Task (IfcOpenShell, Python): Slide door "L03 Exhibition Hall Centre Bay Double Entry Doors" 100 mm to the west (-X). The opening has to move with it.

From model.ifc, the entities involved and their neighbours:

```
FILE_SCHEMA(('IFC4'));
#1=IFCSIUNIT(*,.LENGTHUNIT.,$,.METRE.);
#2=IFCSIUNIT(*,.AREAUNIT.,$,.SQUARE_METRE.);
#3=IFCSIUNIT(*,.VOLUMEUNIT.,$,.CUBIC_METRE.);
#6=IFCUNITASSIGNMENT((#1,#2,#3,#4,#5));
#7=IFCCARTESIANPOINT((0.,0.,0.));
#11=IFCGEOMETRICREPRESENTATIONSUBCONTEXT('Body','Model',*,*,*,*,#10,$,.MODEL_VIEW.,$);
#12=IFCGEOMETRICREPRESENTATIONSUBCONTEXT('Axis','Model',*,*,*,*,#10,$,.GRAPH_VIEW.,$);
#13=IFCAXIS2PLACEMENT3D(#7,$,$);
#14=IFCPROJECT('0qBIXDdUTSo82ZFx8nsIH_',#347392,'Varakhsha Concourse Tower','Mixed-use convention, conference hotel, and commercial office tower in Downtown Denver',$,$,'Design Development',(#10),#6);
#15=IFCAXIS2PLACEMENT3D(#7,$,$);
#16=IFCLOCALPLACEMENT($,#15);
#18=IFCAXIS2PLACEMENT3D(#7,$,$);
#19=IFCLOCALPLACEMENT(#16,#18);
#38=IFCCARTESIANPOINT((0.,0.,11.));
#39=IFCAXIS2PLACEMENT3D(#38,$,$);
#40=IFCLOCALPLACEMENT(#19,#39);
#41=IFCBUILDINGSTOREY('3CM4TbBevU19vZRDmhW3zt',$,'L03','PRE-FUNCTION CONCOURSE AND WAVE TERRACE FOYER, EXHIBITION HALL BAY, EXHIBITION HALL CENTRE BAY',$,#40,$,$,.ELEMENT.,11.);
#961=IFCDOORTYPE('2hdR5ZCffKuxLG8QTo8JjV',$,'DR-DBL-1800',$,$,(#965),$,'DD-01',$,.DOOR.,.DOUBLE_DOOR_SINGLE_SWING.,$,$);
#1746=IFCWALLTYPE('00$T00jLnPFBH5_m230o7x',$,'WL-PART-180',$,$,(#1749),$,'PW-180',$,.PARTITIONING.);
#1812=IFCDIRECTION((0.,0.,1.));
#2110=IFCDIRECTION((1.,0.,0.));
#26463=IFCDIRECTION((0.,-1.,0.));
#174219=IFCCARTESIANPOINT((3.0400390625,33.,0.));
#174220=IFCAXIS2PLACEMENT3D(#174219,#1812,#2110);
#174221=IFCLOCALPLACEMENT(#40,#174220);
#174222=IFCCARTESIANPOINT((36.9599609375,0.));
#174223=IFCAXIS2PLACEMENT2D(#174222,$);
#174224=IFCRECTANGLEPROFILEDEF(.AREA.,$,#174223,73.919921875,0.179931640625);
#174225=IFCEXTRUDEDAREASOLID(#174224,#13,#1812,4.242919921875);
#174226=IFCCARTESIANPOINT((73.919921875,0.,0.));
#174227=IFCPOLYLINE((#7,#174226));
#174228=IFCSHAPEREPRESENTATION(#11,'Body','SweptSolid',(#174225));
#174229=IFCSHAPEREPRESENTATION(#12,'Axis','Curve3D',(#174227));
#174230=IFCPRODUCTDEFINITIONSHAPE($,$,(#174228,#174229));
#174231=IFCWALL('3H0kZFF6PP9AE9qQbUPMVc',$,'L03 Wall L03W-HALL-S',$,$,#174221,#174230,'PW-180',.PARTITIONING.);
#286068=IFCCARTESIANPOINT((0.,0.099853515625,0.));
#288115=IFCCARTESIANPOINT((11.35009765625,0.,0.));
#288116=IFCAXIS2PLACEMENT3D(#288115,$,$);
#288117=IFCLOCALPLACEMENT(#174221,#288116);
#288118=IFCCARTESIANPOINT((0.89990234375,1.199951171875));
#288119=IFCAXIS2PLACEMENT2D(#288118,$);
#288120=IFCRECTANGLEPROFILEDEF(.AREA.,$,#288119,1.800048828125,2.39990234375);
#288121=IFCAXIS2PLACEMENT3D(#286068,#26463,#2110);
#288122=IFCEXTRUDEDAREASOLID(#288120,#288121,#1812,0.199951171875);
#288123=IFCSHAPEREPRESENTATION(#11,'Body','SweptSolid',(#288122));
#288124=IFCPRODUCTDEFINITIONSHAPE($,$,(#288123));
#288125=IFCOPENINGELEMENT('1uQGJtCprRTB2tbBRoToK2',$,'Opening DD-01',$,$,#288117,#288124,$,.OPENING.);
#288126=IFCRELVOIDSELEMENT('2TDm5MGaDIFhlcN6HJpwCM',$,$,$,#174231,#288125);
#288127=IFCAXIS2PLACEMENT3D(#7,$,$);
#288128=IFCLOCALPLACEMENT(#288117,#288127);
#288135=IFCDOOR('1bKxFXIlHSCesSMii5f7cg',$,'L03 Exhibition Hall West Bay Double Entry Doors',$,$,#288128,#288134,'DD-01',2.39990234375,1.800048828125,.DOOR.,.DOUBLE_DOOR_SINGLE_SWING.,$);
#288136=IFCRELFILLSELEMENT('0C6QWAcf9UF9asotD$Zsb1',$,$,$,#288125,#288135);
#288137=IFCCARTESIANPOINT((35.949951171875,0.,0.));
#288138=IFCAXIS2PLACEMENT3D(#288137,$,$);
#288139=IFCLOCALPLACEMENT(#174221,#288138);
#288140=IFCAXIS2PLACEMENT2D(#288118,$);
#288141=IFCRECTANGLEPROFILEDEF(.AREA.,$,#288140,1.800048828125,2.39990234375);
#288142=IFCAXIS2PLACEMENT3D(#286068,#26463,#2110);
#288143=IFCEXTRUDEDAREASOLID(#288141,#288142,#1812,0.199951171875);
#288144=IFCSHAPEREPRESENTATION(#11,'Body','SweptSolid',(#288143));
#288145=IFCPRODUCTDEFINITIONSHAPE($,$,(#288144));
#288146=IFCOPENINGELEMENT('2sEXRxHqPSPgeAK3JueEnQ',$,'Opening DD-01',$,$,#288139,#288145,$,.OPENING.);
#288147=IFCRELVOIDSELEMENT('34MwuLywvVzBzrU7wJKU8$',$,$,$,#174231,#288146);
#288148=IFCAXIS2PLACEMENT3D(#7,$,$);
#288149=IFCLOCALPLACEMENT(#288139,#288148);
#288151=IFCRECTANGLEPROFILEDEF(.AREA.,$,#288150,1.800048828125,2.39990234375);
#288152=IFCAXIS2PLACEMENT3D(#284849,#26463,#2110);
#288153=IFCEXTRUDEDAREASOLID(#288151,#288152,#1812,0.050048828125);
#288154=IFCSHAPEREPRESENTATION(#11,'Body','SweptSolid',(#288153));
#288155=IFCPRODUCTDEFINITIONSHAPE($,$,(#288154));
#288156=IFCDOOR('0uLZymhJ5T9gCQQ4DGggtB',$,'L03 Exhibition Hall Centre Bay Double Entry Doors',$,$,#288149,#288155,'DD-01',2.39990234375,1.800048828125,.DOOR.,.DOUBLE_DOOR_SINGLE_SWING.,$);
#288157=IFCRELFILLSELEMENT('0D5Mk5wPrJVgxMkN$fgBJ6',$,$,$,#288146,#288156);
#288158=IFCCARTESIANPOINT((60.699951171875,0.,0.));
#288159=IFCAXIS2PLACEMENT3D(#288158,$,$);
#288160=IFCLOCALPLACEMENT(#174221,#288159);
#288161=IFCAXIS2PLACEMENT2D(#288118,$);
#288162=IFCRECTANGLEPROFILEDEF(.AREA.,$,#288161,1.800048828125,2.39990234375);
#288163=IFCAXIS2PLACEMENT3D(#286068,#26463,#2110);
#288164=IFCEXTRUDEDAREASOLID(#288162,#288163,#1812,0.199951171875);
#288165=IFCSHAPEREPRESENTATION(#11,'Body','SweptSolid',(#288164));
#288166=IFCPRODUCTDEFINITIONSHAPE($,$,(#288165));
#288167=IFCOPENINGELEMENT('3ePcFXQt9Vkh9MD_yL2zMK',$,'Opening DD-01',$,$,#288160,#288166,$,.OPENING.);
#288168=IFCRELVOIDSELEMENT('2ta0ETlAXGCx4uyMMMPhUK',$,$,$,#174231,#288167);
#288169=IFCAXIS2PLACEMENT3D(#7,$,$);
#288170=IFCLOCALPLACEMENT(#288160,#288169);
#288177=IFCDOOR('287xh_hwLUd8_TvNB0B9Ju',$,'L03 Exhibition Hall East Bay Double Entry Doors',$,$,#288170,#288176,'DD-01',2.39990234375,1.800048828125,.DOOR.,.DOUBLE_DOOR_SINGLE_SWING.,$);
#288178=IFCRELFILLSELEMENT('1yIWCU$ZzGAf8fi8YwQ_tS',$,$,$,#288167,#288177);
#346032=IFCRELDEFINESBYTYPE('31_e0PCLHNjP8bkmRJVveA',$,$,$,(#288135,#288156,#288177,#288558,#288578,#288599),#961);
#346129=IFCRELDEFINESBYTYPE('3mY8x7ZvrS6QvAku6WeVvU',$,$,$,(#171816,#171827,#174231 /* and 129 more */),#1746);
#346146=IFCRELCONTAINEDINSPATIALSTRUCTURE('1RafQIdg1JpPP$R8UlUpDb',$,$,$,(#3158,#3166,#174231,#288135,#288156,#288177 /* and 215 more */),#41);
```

```python
import ifcopenshell
import ifcopenshell.api.geometry
import ifcopenshell.util.placement
import ifcopenshell.util.unit

model = ifcopenshell.open("model.ifc")
unit_scale = ifcopenshell.util.unit.calculate_unit_scale(model)

door = model.by_guid("0uLZymhJ5T9gCQQ4DGggtB")
opening = door.FillsVoids[0].RelatingOpeningElement
wall = opening.VoidsElements[0].RelatingBuildingElement

wall_matrix = ifcopenshell.util.placement.get_local_placement(wall.ObjectPlacement)
shift = wall_matrix[:3, 0] * -0.1 / unit_scale
before = ifcopenshell.util.placement.get_local_placement(door.ObjectPlacement)[:3, 3].copy()

# The door is placed relative to its opening, so it follows when the opening moves.
matrix = ifcopenshell.util.placement.get_local_placement(opening.ObjectPlacement)
matrix[:3, 3] += shift
ifcopenshell.api.geometry.edit_object_placement(
    model, product=opening, matrix=matrix, is_si=False, should_transform_children=True
)

after = ifcopenshell.util.placement.get_local_placement(door.ObjectPlacement)[:3, 3]
print("door moved by", (after - before).round(3) + 0.0)

model.write("model_rev.ifc")
```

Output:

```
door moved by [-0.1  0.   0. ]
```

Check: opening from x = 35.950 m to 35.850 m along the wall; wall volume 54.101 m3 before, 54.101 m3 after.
